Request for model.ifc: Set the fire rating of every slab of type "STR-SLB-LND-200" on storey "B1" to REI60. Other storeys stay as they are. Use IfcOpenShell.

First a look at what the model holds.

```python
import ifcopenshell
import ifcopenshell.util.element

model = ifcopenshell.open("model.ifc")
print(model.schema)
storey = next(s for s in model.by_type("IfcBuildingStorey") if s.Name == "B1")
slabs = [e for e in ifcopenshell.util.element.get_decomposition(storey) if e.is_a("IfcSlab")]
seen = {}
for e in slabs:
    element_type = ifcopenshell.util.element.get_type(e)
    key = (element_type.Name if element_type != e and element_type else None, ifcopenshell.util.element.get_pset(e, "Pset_SlabCommon", "FireRating"))
    seen[key] = seen.get(key, 0) + 1
for (name, value), count in sorted(seen.items(), key=str):
    print(count, "x", name, "|", value)
```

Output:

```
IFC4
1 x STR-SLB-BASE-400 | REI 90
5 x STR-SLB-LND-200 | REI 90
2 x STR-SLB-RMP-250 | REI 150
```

```python
import ifcopenshell
import ifcopenshell.api.pset
import ifcopenshell.util.element

model = ifcopenshell.open("model.ifc")

storey = next(s for s in model.by_type("IfcBuildingStorey") if s.Name == "B1")
slabs = [e for e in ifcopenshell.util.element.get_decomposition(storey) if e.is_a("IfcSlab")]

count = 0
for e in slabs:
    element_type = ifcopenshell.util.element.get_type(e)
    if element_type in (None, e) or element_type.Name != "STR-SLB-LND-200":
        continue
    # add_pset returns the element's existing set when there is one.
    pset = ifcopenshell.api.pset.add_pset(model, product=e, name="Pset_SlabCommon")
    ifcopenshell.api.pset.edit_pset(model, pset=pset, properties={"FireRating": "REI60"})
    count += 1

print(count, "slabs updated")

model.write("model_v2.ifc")
```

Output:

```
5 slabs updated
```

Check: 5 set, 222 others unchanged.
